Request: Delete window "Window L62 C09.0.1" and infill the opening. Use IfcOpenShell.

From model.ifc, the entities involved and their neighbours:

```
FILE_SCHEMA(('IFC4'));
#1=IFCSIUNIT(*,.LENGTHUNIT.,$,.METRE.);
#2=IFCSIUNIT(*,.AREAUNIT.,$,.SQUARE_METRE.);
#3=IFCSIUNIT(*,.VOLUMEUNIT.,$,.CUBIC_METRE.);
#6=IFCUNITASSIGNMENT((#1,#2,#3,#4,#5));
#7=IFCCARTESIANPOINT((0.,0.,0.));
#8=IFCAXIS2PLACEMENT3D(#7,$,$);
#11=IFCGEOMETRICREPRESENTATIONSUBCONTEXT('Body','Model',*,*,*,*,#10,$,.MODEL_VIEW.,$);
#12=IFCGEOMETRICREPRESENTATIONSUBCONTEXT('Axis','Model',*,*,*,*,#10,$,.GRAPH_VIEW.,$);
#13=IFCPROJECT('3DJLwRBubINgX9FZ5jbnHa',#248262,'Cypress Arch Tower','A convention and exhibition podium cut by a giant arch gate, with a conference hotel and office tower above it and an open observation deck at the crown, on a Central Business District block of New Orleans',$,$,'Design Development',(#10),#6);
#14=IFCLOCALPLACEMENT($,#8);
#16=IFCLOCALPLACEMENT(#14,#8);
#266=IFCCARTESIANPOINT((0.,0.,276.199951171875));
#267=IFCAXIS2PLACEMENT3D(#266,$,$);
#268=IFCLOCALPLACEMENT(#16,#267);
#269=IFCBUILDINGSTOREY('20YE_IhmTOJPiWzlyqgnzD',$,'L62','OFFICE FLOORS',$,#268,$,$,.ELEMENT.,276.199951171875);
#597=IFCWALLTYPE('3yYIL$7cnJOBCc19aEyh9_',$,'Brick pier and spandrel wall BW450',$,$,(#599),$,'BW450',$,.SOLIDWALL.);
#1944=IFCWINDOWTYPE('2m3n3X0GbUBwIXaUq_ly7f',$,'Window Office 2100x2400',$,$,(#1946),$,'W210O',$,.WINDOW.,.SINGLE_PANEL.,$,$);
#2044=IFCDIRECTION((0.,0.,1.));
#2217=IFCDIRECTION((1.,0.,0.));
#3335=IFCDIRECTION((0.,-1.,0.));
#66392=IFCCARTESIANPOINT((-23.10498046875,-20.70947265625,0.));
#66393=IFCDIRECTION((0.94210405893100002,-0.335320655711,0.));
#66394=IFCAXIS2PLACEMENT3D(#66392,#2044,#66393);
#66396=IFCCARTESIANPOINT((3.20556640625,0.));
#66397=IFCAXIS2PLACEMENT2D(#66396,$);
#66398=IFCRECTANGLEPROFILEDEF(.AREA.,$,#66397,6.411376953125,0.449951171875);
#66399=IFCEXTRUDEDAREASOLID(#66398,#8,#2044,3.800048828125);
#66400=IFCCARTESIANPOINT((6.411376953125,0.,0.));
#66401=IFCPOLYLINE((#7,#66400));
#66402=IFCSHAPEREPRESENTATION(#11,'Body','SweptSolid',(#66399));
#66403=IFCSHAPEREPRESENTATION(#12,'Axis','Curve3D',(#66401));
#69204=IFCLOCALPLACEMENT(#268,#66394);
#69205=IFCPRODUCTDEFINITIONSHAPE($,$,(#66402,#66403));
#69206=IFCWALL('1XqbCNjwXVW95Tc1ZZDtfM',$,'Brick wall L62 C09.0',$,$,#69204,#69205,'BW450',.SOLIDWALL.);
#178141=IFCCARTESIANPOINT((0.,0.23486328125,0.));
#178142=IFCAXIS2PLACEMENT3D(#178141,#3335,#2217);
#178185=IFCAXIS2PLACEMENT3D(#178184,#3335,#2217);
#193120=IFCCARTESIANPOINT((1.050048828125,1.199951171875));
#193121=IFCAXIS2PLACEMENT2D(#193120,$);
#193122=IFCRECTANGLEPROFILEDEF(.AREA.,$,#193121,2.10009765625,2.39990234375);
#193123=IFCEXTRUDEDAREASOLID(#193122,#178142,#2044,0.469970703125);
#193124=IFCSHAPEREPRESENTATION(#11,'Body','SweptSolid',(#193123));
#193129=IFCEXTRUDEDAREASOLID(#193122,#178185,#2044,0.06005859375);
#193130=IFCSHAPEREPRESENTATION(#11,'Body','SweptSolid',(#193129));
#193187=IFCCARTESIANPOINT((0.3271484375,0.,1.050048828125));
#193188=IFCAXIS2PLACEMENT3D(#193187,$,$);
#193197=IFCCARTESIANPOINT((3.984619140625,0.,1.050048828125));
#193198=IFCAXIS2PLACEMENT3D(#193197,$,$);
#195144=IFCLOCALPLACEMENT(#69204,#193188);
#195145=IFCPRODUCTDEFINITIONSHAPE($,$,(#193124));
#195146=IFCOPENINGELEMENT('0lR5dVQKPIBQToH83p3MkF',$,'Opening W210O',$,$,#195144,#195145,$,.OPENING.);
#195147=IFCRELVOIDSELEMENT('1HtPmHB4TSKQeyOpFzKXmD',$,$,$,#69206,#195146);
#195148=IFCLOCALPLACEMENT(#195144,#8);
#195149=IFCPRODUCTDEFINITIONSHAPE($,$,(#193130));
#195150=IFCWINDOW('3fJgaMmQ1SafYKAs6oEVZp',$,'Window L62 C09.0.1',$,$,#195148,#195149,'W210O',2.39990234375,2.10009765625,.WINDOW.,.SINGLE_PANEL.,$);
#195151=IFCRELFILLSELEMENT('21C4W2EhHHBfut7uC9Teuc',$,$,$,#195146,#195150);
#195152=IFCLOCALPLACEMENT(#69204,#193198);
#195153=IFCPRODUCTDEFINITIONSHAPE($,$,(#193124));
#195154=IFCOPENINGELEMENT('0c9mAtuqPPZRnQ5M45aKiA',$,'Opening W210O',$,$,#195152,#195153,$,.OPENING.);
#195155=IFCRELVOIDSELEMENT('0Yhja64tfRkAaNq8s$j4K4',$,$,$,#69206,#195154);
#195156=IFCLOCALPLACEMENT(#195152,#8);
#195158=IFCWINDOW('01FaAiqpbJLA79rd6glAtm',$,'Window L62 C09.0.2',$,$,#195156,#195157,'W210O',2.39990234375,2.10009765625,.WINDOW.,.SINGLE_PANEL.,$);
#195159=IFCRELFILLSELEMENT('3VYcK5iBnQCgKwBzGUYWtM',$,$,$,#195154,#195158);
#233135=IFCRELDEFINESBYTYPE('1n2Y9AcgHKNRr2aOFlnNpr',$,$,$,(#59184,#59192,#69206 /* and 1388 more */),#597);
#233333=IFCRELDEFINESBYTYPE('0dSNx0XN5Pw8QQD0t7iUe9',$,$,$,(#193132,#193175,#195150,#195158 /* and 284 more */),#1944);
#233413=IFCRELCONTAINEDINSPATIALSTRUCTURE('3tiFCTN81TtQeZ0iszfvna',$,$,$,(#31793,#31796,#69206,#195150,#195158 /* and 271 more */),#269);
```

```python
import ifcopenshell
import ifcopenshell.api.feature
import ifcopenshell.api.root
import ifcopenshell.geom
import ifcopenshell.util.shape

model = ifcopenshell.open("model.ifc")
settings = ifcopenshell.geom.settings()


def volume(element):
    """Net volume in cubic metres, openings subtracted."""
    shape = ifcopenshell.geom.create_shape(settings, element)
    return ifcopenshell.util.shape.get_volume(shape.geometry)


window = model.by_id(195150)
opening = window.FillsVoids[0].RelatingOpeningElement
wall = opening.VoidsElements[0].RelatingBuildingElement
before = volume(wall)

ifcopenshell.api.root.remove_product(model, product=window)
ifcopenshell.api.feature.remove_feature(model, feature=opening)

after = volume(wall)

print(f"wall volume {before:.3f} -> {after:.3f} m3")

model.write("model_edited.ifc")
```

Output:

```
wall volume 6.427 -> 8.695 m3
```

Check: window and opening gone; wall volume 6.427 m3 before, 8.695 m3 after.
